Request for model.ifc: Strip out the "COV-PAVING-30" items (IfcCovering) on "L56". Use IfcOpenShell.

First a look at what the model holds.

```python
import ifcopenshell
import ifcopenshell.util.element

model = ifcopenshell.open("model.ifc")
print(model.schema)
storey = next(s for s in model.by_type("IfcBuildingStorey") if s.Name == "L56")
coverings = [e for e in ifcopenshell.util.element.get_decomposition(storey) if e.is_a("IfcCovering")]
seen = {}
for e in coverings:
    element_type = ifcopenshell.util.element.get_type(e)
    name = element_type.Name if element_type not in (None, e) else None
    seen[name] = seen.get(name, 0) + 1
for name, count in sorted(seen.items(), key=str):
    print(count, "x", name)
```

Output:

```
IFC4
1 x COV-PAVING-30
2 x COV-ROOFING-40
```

```python
import ifcopenshell
import ifcopenshell.api.root
import ifcopenshell.util.element

model = ifcopenshell.open("model.ifc")

storey = next(s for s in model.by_type("IfcBuildingStorey") if s.Name == "L56")
coverings = [e for e in ifcopenshell.util.element.get_decomposition(storey) if e.is_a("IfcCovering")]
targets = [e for e in coverings if (t := ifcopenshell.util.element.get_type(e)) not in (None, e) and t.Name == "COV-PAVING-30"]

for e in targets:
    ifcopenshell.api.root.remove_product(model, product=e)
print(len(targets), "removed")

model.write("model_rev.ifc")
```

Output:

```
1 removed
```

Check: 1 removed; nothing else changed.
